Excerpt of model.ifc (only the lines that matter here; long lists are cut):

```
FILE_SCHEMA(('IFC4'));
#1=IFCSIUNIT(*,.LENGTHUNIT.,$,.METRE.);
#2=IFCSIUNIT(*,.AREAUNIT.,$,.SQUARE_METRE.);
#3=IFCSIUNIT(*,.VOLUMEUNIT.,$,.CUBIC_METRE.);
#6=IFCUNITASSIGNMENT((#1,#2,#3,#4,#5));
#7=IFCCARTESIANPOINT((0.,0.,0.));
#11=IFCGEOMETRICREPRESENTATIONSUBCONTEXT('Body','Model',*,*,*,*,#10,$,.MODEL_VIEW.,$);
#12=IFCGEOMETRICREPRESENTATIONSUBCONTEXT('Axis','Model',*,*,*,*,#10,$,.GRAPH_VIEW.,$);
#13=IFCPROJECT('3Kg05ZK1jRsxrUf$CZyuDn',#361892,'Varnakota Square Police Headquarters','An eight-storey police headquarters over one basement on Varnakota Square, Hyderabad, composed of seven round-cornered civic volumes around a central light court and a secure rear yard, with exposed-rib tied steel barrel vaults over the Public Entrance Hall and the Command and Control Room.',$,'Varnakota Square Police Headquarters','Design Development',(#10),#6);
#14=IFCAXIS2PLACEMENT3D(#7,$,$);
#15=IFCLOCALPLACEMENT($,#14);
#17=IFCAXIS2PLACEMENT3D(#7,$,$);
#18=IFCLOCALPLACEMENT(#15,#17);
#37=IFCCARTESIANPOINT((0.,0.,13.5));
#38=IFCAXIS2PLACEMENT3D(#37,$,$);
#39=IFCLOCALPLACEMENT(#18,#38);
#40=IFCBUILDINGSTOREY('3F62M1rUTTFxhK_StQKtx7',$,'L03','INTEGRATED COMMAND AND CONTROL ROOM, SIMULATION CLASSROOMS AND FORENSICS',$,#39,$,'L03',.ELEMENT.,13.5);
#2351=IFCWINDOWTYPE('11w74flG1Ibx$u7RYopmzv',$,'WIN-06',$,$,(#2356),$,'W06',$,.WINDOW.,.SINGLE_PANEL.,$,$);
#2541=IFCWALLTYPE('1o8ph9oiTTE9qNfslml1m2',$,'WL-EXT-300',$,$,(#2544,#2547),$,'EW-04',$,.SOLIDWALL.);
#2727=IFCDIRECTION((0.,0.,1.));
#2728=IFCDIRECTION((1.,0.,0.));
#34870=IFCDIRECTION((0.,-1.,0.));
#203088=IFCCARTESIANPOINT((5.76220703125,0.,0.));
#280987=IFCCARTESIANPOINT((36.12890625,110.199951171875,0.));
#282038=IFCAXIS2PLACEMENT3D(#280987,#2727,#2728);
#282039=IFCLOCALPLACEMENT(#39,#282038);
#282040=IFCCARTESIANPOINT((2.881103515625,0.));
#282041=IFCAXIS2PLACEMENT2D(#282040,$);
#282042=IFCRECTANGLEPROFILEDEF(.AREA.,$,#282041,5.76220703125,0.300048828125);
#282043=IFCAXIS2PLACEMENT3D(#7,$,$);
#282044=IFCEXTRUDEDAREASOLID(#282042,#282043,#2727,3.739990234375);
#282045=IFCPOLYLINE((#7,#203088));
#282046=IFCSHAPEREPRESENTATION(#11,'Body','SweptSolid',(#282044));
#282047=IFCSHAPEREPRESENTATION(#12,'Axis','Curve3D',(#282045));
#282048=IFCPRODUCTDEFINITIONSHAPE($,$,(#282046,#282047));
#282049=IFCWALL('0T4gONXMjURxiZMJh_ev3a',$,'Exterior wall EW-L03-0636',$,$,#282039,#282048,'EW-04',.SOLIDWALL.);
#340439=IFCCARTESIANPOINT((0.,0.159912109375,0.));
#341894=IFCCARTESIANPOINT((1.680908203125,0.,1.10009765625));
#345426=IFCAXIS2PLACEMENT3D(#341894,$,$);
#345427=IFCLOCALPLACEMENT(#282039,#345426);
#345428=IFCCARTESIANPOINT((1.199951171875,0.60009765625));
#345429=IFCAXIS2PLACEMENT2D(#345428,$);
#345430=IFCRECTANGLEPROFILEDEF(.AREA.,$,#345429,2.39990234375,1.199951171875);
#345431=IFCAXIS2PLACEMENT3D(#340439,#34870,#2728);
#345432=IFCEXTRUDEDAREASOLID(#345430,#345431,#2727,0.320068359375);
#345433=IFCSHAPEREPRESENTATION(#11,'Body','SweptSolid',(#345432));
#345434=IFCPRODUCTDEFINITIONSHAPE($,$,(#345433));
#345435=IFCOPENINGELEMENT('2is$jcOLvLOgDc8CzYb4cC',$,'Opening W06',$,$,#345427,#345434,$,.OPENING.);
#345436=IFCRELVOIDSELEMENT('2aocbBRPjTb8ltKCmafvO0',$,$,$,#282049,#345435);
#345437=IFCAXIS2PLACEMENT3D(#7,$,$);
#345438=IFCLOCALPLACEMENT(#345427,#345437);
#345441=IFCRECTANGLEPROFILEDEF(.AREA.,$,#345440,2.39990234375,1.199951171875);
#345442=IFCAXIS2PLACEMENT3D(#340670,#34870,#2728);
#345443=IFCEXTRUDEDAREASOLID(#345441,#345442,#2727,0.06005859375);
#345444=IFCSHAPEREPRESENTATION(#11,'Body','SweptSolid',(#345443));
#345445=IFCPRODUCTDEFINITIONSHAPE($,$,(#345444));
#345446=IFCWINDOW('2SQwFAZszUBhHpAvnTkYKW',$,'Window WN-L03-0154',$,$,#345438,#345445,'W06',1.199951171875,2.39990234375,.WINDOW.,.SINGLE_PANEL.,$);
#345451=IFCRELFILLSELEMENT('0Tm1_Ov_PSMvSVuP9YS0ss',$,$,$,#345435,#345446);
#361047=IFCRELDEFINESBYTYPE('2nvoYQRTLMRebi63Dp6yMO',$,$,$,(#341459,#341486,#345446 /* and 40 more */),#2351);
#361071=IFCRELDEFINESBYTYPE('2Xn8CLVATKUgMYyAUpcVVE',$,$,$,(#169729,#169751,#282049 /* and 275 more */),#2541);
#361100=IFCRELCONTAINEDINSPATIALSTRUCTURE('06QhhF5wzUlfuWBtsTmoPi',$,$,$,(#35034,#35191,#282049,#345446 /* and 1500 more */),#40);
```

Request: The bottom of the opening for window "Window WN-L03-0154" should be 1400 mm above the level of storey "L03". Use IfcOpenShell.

```python
import numpy as np
import ifcopenshell
import ifcopenshell.api.geometry
import ifcopenshell.geom
import ifcopenshell.util.element
import ifcopenshell.util.placement
import ifcopenshell.util.shape
import ifcopenshell.util.unit

model = ifcopenshell.open("model.ifc")
unit_scale = ifcopenshell.util.unit.calculate_unit_scale(model)

window = model.by_guid("2SQwFAZszUBhHpAvnTkYKW")
opening = window.FillsVoids[0].RelatingOpeningElement
storey = ifcopenshell.util.element.get_container(window, ifc_class="IfcBuildingStorey")
level = ifcopenshell.util.placement.get_local_placement(storey.ObjectPlacement)[2, 3]

# The opening's origin need not be at the sill, so measure its lowest point.
shape = ifcopenshell.geom.create_shape(ifcopenshell.geom.settings(), opening)
bottom = ifcopenshell.util.shape.get_shape_bottom_elevation(shape, shape.geometry) / unit_scale
dz = level + 1.4 / unit_scale - bottom

shift = np.array([0.0, 0.0, dz])
# The window is placed relative to its opening, so it follows when the opening moves.
matrix = ifcopenshell.util.placement.get_local_placement(opening.ObjectPlacement)
matrix[:3, 3] += shift
ifcopenshell.api.geometry.edit_object_placement(
    model, product=opening, matrix=matrix, is_si=False, should_transform_children=True
)

print(f"moved by {dz * unit_scale:+.3f} m")

model.write("model_v2.ifc")
```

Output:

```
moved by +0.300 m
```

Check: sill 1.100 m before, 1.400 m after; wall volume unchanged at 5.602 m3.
